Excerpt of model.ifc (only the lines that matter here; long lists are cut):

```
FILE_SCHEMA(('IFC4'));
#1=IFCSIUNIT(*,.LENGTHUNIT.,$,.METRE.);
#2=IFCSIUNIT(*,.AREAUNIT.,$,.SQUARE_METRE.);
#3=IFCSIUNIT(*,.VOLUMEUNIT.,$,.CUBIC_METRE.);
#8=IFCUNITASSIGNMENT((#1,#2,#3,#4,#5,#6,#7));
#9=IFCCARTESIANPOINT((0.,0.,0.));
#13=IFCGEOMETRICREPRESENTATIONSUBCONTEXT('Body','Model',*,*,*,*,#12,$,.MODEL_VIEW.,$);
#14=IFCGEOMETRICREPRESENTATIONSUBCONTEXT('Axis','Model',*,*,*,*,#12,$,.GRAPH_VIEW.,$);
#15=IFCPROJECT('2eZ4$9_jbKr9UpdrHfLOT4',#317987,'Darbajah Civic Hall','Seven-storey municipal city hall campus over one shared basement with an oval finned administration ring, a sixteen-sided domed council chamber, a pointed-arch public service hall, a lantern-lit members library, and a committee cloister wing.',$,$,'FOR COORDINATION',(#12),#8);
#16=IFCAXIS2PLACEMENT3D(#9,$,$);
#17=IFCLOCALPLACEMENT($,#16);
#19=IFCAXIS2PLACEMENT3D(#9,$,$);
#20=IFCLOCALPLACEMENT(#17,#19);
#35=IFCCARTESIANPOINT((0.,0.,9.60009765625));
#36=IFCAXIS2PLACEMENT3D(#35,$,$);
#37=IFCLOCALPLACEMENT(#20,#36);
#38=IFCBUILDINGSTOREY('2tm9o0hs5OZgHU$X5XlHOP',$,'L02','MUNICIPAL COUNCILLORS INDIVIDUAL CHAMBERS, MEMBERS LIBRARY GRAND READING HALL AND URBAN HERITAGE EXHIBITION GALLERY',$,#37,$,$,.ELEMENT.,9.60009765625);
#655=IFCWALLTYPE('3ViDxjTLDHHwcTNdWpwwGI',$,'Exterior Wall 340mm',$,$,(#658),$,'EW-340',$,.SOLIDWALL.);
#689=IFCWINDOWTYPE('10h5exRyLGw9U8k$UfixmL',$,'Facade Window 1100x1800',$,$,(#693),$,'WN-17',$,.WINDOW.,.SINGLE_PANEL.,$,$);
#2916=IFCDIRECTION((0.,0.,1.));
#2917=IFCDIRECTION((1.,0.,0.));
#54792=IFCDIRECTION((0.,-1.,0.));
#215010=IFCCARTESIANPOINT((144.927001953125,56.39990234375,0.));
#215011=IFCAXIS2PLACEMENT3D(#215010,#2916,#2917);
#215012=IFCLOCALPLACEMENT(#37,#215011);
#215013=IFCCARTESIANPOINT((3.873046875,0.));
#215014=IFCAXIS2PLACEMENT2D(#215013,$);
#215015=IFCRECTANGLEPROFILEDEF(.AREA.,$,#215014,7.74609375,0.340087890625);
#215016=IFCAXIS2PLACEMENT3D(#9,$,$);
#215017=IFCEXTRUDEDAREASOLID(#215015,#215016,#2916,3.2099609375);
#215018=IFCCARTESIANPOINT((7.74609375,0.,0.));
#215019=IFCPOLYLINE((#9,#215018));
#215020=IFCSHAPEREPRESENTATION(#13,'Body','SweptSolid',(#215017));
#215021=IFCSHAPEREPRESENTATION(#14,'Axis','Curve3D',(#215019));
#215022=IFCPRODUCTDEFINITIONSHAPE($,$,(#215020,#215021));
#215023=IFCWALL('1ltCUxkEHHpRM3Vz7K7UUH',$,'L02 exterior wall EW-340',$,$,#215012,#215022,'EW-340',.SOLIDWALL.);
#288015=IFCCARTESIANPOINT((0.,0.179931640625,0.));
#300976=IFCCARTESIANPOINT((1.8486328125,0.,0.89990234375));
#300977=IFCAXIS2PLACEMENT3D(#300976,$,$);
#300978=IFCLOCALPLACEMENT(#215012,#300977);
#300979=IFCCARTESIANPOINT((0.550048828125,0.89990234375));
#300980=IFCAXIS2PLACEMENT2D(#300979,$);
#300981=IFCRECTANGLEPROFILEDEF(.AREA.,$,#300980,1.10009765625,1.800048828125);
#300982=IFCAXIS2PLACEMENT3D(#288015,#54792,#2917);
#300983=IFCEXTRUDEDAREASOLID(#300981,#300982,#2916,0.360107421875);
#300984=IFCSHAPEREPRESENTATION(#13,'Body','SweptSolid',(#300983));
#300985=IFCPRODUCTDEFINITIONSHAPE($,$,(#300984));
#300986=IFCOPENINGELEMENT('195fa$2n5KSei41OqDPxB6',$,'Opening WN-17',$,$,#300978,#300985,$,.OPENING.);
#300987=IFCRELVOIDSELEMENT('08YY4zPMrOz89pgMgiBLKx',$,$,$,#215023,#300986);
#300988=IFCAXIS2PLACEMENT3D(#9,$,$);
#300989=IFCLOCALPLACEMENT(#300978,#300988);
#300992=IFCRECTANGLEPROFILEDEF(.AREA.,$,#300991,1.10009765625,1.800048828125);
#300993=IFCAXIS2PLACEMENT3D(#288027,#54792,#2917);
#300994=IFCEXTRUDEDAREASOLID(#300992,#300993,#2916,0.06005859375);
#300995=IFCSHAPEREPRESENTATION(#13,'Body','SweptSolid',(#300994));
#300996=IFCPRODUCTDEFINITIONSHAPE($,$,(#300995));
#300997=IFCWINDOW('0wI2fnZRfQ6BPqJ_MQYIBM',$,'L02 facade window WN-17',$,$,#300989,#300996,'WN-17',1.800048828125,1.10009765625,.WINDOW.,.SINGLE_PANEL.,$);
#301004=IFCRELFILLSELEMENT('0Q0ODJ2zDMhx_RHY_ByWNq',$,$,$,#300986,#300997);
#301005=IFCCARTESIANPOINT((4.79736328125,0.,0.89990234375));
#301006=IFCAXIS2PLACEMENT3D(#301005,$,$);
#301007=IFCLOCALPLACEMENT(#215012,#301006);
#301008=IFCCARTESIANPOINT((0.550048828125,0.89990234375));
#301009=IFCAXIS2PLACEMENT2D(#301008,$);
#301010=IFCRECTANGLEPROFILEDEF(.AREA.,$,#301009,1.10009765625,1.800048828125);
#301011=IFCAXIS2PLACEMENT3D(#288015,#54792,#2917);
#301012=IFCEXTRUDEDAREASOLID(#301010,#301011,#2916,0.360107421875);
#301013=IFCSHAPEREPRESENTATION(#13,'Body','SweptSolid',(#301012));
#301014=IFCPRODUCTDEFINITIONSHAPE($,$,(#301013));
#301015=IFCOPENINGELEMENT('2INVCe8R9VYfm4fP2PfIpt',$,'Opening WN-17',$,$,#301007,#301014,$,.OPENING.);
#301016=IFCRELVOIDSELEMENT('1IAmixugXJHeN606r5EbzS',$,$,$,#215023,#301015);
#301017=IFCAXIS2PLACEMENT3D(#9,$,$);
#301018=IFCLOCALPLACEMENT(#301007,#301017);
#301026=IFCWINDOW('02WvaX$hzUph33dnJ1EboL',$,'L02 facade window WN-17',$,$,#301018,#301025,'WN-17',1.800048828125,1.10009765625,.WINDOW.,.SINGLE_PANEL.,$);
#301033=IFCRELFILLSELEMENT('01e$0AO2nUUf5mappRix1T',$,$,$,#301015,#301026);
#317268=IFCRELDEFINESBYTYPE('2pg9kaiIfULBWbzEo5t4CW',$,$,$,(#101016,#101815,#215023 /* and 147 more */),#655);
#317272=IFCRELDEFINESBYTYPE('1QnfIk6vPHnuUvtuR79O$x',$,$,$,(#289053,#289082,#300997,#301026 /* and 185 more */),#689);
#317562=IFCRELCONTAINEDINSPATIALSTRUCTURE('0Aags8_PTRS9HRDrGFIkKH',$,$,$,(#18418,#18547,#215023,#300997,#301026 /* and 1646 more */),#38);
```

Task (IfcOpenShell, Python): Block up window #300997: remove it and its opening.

```python
import ifcopenshell
import ifcopenshell.api.feature
import ifcopenshell.api.root
import ifcopenshell.geom
import ifcopenshell.util.shape

model = ifcopenshell.open("model.ifc")
settings = ifcopenshell.geom.settings()


def volume(element):
    """Net volume in cubic metres, openings subtracted."""
    shape = ifcopenshell.geom.create_shape(settings, element)
    return ifcopenshell.util.shape.get_volume(shape.geometry)


window = model.by_guid("0wI2fnZRfQ6BPqJ_MQYIBM")
opening = window.FillsVoids[0].RelatingOpeningElement
wall = opening.VoidsElements[0].RelatingBuildingElement
before = volume(wall)

ifcopenshell.api.root.remove_product(model, product=window)
ifcopenshell.api.feature.remove_feature(model, feature=opening)

after = volume(wall)

print(f"wall volume {before:.3f} -> {after:.3f} m3")

model.write("model_edited.ifc")
```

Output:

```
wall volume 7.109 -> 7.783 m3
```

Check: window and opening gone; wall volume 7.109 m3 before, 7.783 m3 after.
